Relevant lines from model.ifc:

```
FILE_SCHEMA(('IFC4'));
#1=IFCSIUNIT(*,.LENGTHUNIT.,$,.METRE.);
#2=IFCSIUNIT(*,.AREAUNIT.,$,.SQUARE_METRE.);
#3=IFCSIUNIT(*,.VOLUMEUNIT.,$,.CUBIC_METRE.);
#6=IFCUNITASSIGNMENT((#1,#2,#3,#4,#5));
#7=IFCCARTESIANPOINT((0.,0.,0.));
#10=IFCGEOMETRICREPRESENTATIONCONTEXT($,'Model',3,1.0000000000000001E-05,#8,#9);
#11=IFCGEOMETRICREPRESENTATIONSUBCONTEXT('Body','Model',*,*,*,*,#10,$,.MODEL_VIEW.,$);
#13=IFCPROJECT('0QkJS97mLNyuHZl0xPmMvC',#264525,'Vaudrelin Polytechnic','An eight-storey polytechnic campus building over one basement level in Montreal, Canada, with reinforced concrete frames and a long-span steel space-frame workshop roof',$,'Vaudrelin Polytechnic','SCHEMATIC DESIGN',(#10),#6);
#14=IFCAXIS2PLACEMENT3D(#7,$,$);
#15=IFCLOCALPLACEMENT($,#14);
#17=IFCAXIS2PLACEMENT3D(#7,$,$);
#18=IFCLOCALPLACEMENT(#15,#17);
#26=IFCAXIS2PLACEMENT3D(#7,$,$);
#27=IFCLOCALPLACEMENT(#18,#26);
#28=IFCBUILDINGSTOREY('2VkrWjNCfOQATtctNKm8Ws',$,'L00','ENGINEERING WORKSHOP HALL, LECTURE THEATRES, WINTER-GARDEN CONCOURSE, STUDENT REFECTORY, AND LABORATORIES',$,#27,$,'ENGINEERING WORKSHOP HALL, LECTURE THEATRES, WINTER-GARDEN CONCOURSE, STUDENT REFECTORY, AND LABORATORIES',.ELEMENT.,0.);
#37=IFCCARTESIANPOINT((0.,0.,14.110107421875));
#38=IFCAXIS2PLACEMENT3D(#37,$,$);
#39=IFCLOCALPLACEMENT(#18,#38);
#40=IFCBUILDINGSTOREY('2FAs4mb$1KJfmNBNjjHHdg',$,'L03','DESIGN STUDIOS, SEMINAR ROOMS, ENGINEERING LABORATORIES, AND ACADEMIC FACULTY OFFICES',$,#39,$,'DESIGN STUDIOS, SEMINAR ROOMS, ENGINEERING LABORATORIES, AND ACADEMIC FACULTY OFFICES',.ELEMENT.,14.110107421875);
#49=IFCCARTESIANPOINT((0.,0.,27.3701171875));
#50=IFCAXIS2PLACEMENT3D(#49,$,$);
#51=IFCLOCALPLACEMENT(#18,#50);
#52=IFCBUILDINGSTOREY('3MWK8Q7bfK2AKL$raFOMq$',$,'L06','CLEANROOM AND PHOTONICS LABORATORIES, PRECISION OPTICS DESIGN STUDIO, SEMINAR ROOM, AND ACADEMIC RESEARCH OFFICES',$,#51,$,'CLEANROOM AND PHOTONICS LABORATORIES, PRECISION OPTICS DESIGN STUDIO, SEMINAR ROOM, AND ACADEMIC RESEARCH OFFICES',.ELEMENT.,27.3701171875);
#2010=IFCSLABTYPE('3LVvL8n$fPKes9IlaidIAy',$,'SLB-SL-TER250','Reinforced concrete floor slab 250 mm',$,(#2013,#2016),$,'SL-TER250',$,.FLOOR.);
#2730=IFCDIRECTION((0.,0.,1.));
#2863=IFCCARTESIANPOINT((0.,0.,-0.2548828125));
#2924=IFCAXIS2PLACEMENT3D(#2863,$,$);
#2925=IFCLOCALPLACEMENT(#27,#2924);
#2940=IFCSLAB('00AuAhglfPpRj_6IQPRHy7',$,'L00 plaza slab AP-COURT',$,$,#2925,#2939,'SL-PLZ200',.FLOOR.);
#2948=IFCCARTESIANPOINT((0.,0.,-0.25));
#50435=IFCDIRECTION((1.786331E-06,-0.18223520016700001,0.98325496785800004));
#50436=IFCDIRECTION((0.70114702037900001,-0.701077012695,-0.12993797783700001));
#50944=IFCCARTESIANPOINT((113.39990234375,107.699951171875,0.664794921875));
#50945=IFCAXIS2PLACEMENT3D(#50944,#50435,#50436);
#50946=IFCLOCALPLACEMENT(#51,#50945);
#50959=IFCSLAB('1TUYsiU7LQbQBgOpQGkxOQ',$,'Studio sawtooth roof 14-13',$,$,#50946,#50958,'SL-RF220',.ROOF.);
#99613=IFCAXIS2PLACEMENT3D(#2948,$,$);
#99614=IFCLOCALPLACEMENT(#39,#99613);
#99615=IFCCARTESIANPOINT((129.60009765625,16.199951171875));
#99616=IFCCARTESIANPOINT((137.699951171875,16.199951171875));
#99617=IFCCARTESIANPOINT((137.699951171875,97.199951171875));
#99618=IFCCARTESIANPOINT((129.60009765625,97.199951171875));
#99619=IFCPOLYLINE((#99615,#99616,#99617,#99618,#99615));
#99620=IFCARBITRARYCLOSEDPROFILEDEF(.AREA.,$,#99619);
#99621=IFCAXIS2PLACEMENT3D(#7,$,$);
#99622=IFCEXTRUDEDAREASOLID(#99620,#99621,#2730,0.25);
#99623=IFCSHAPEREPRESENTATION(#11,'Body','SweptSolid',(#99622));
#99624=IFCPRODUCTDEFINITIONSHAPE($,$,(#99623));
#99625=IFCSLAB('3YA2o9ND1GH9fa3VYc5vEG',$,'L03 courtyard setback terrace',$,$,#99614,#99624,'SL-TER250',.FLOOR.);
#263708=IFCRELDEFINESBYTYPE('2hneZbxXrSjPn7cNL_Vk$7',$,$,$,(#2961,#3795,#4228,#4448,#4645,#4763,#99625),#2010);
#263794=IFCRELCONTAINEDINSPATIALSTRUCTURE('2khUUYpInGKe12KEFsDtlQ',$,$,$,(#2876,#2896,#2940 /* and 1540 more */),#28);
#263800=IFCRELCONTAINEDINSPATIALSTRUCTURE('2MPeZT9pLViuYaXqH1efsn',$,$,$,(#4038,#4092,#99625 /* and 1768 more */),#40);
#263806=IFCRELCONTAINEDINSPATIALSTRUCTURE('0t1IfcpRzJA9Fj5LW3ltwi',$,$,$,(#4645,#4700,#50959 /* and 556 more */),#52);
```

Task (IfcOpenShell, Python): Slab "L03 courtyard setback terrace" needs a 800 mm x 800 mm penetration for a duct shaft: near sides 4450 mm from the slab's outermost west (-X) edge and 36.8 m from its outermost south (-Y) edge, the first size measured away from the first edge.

```python
import numpy as np
import ifcopenshell
import ifcopenshell.api.feature
import ifcopenshell.api.geometry
import ifcopenshell.api.root
import ifcopenshell.geom
import ifcopenshell.util.placement
import ifcopenshell.util.representation
import ifcopenshell.util.shape
import ifcopenshell.util.unit

model = ifcopenshell.open("model.ifc")
unit_scale = ifcopenshell.util.unit.calculate_unit_scale(model)
settings = ifcopenshell.geom.settings()


def volume(element):
    """Net volume in cubic metres, openings subtracted."""
    shape = ifcopenshell.geom.create_shape(settings, element)
    return ifcopenshell.util.shape.get_volume(shape.geometry)


slab = model.by_id(99625)
before = volume(slab)

# Extent in the slab's own axes, in metres. The edges named are its -X and -Y sides.
slab_shape = ifcopenshell.geom.create_shape(settings, slab)
vertices = ifcopenshell.util.shape.get_vertices(slab_shape.geometry)
x_min, y_min, bottom = vertices.min(axis=0)
top = vertices[:, 2].max()

opening = ifcopenshell.api.root.create_entity(model, ifc_class="IfcOpeningElement", name="Duct shaft opening", predefined_type="OPENING")
context = ifcopenshell.util.representation.get_context(model, "Model", "Body", "MODEL_VIEW")
width, depth = 0.8, 0.8
outline = [(0.0, 0.0), (width, 0.0), (width, depth), (0.0, depth), (0.0, 0.0)]
# Overshoot both faces by 50 mm so the cut is clean.
shape = ifcopenshell.api.geometry.add_slab_representation(
    model, context=context, depth=top - bottom + 0.1, polyline=outline
)
ifcopenshell.api.geometry.assign_representation(model, product=opening, representation=shape)

matrix = ifcopenshell.util.placement.get_local_placement(slab.ObjectPlacement)
matrix[:, 3] = matrix @ np.append(np.array([x_min + 4.45, y_min + 36.8, bottom - 0.05]) / unit_scale, 1.0)
ifcopenshell.api.geometry.edit_object_placement(model, product=opening, matrix=matrix, is_si=False)
ifcopenshell.api.feature.add_feature(model, feature=opening, element=slab)

after = volume(slab)

print(f"slab volume {before:.3f} -> {after:.3f} m3")

model.write("model_rev.ifc")
```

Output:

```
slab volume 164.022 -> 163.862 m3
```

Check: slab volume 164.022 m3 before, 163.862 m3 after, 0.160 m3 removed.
